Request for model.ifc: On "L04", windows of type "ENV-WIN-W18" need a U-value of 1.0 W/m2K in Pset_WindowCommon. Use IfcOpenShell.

First a look at what the model holds.

```python
import ifcopenshell
import ifcopenshell.util.element

model = ifcopenshell.open("model.ifc")
print(model.schema)
storey = next(s for s in model.by_type("IfcBuildingStorey") if s.Name == "L04")
windows = [e for e in ifcopenshell.util.element.get_decomposition(storey) if e.is_a("IfcWindow")]
seen = {}
for e in windows:
    element_type = ifcopenshell.util.element.get_type(e)
    key = (element_type.Name if element_type != e and element_type else None, ifcopenshell.util.element.get_pset(e, "Pset_WindowCommon", "ThermalTransmittance"))
    seen[key] = seen.get(key, 0) + 1
for (name, value), count in sorted(seen.items(), key=str):
    print(count, "x", name, "|", value)
```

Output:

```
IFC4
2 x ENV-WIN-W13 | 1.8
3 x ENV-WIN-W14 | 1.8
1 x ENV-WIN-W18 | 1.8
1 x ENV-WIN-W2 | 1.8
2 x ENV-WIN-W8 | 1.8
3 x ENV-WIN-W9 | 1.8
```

```python
import ifcopenshell
import ifcopenshell.api.pset
import ifcopenshell.util.element

model = ifcopenshell.open("model.ifc")

storey = next(s for s in model.by_type("IfcBuildingStorey") if s.Name == "L04")
windows = [e for e in ifcopenshell.util.element.get_decomposition(storey) if e.is_a("IfcWindow")]

count = 0
for e in windows:
    element_type = ifcopenshell.util.element.get_type(e)
    if element_type in (None, e) or element_type.Name != "ENV-WIN-W18":
        continue
    # add_pset returns the element's existing set when there is one.
    pset = ifcopenshell.api.pset.add_pset(model, product=e, name="Pset_WindowCommon")
    ifcopenshell.api.pset.edit_pset(model, pset=pset, properties={"ThermalTransmittance": 1.0})
    count += 1

print(count, "windows updated")

model.write("model_rev.ifc")
```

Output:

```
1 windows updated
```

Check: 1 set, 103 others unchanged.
